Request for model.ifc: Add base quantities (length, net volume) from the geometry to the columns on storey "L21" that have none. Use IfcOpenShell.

First a look at what the model holds.

```python
import ifcopenshell
import ifcopenshell.util.element
import ifcopenshell.util.unit

model = ifcopenshell.open("model.ifc")
print(model.schema)
for unit_type in ("LENGTHUNIT", "AREAUNIT", "VOLUMEUNIT"):
    print(unit_type, ifcopenshell.util.unit.calculate_unit_scale(model, unit_type))
storey = next(s for s in model.by_type("IfcBuildingStorey") if s.Name == "L21")
columns = [e for e in ifcopenshell.util.element.get_decomposition(storey) if e.is_a("IfcColumn")]
for e in sorted(columns, key=lambda e: e.id()):
    print(e.id(), e.is_a(), e.Name, list(ifcopenshell.util.element.get_psets(e, qtos_only=True)), sep=" | ")
```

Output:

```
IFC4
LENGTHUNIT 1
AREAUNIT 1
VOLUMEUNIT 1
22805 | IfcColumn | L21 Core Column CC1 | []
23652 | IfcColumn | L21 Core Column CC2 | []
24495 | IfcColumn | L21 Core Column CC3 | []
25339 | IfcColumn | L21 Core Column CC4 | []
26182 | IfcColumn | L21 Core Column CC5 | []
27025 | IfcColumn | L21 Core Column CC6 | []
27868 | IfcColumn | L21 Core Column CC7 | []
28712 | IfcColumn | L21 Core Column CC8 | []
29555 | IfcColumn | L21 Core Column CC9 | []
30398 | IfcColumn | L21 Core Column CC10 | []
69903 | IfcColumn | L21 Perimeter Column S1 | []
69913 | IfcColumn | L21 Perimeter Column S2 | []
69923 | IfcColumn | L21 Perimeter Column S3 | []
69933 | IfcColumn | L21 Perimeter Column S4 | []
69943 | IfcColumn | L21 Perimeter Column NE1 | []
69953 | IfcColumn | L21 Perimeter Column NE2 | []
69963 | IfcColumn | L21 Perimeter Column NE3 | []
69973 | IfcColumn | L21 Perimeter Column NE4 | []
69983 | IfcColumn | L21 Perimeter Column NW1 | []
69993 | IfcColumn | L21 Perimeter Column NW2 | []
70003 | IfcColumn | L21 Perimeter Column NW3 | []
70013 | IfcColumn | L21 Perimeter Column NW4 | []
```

```python
import ifcopenshell
import ifcopenshell.api.pset
import ifcopenshell.geom
import ifcopenshell.util.element
import ifcopenshell.util.shape
import ifcopenshell.util.unit

model = ifcopenshell.open("model.ifc")
unit_scale = ifcopenshell.util.unit.calculate_unit_scale(model)
volume_scale = ifcopenshell.util.unit.calculate_unit_scale(model, "VOLUMEUNIT")
settings = ifcopenshell.geom.settings()

storey = next(s for s in model.by_type("IfcBuildingStorey") if s.Name == "L21")
columns = [e for e in ifcopenshell.util.element.get_decomposition(storey) if e.is_a("IfcColumn")]

for e in sorted(columns, key=lambda e: e.id()):
    if ifcopenshell.util.element.get_psets(e, qtos_only=True, should_inherit=False):
        continue
    # Geometry comes back in metres, in the element's own axes.
    shape = ifcopenshell.geom.create_shape(settings, e)
    values = {
        "Length": ifcopenshell.util.shape.get_z(shape.geometry) / unit_scale,
        "NetVolume": ifcopenshell.util.shape.get_volume(shape.geometry) / volume_scale,
    }
    qto = ifcopenshell.api.pset.add_qto(model, product=e, name="Qto_ColumnBaseQuantities")
    ifcopenshell.api.pset.edit_qto(model, qto=qto, properties=values)
    print(e.id(), {k: round(v, 3) for k, v in values.items()})

model.write("model_edited.ifc")
```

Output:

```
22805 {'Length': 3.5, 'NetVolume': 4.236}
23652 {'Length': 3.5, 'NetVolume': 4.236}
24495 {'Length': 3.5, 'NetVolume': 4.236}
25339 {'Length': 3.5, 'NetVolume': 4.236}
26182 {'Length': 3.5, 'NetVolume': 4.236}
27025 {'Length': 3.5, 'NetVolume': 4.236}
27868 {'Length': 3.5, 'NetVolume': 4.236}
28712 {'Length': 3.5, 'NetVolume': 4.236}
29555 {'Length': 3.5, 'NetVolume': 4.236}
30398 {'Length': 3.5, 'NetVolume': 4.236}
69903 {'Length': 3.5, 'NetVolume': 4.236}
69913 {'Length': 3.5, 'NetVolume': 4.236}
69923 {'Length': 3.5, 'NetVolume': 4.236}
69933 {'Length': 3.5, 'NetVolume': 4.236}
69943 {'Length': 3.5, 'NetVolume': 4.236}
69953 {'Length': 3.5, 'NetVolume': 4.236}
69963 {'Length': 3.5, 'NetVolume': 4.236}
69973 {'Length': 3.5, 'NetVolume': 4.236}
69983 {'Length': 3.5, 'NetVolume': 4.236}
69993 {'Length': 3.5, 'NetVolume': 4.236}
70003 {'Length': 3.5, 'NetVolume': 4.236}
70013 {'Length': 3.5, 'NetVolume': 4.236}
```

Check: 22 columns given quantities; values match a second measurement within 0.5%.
